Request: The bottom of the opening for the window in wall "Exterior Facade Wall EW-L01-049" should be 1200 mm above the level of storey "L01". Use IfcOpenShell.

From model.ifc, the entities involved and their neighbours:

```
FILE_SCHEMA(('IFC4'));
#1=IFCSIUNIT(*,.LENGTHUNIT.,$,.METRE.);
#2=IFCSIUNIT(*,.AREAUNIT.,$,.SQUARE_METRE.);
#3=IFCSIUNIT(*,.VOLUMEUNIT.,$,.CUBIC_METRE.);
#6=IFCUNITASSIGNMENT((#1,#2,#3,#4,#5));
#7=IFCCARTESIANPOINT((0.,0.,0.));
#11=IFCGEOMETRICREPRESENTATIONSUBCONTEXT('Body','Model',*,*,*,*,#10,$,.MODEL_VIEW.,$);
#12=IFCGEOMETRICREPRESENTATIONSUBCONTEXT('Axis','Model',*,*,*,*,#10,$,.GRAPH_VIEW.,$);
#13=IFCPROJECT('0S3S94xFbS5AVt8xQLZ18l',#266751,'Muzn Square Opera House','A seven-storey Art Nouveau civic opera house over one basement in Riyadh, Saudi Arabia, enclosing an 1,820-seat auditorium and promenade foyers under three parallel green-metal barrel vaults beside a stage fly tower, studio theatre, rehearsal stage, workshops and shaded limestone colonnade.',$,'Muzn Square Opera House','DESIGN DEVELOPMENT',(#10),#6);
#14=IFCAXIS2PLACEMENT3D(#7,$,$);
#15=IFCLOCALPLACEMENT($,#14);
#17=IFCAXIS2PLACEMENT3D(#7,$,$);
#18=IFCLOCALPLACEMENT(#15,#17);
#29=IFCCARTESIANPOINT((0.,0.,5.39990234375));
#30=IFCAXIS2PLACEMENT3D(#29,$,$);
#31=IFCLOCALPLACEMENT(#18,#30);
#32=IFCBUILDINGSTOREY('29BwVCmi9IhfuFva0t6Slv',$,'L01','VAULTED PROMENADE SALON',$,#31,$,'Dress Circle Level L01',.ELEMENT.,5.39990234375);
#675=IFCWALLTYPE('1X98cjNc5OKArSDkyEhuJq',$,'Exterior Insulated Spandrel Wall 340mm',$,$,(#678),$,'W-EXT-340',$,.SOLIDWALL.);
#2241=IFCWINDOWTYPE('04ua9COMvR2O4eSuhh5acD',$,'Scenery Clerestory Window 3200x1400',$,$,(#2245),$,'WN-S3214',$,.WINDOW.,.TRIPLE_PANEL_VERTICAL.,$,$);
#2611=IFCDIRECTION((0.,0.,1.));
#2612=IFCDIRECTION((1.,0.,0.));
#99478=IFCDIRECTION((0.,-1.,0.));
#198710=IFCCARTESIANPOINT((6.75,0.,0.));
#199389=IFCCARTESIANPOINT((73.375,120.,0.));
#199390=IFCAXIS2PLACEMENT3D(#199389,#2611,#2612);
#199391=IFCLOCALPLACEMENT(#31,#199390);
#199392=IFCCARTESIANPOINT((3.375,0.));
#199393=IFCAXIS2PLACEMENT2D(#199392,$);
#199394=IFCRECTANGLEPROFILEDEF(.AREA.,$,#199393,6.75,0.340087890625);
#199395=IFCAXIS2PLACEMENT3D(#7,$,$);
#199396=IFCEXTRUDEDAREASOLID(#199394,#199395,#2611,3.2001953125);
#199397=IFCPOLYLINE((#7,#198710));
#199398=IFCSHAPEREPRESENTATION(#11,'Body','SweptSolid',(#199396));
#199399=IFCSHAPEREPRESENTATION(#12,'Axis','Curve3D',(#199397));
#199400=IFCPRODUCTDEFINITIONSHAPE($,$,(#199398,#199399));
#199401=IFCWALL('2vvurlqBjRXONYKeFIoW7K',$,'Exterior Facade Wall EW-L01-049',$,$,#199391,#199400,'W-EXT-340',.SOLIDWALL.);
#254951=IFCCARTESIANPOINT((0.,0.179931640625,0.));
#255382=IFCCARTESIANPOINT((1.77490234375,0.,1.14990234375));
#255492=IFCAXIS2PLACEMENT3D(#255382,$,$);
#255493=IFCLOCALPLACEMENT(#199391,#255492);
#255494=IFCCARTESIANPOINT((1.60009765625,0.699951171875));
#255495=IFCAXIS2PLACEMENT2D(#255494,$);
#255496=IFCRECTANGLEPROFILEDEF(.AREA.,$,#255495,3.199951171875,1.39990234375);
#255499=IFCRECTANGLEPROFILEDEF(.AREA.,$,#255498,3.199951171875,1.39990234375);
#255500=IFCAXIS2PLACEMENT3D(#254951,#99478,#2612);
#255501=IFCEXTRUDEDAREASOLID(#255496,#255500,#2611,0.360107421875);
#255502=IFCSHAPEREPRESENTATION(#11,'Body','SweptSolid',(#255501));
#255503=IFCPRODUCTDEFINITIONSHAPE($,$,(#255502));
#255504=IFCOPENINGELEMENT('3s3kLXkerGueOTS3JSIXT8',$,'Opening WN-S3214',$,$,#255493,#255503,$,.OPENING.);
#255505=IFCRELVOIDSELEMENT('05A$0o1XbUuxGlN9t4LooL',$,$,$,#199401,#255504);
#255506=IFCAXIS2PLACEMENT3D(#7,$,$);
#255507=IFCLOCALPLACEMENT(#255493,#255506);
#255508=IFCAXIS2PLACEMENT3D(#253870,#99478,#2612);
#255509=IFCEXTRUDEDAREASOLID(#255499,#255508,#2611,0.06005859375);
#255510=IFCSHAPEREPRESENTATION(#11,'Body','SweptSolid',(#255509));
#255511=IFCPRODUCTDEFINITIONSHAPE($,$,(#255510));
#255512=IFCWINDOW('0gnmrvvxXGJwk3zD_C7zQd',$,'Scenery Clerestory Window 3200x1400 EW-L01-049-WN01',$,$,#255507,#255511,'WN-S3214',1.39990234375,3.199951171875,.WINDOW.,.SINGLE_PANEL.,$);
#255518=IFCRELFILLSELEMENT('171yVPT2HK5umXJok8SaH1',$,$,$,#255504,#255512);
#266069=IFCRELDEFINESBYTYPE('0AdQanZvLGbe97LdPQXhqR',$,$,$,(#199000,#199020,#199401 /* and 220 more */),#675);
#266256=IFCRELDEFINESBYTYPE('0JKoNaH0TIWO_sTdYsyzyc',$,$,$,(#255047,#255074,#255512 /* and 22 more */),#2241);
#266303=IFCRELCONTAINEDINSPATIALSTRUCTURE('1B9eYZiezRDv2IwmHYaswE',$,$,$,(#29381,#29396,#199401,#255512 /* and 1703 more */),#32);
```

```python
import numpy as np
import ifcopenshell
import ifcopenshell.api.geometry
import ifcopenshell.geom
import ifcopenshell.util.element
import ifcopenshell.util.placement
import ifcopenshell.util.shape
import ifcopenshell.util.unit

model = ifcopenshell.open("model.ifc")
unit_scale = ifcopenshell.util.unit.calculate_unit_scale(model)

window = model.by_id(255512)
opening = window.FillsVoids[0].RelatingOpeningElement
storey = ifcopenshell.util.element.get_container(window, ifc_class="IfcBuildingStorey")
level = ifcopenshell.util.placement.get_local_placement(storey.ObjectPlacement)[2, 3]

# The opening's origin need not be at the sill, so measure its lowest point.
shape = ifcopenshell.geom.create_shape(ifcopenshell.geom.settings(), opening)
bottom = ifcopenshell.util.shape.get_shape_bottom_elevation(shape, shape.geometry) / unit_scale
dz = level + 1.2 - bottom

shift = np.array([0.0, 0.0, dz])
# The window is placed relative to its opening, so it follows when the opening moves.
matrix = ifcopenshell.util.placement.get_local_placement(opening.ObjectPlacement)
matrix[:3, 3] += shift
ifcopenshell.api.geometry.edit_object_placement(
    model, product=opening, matrix=matrix, is_si=False, should_transform_children=True
)

print(f"moved by {dz * unit_scale:+.3f} m")

model.write("model_rev.ifc")
```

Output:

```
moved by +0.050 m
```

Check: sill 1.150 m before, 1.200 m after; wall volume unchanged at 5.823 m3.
